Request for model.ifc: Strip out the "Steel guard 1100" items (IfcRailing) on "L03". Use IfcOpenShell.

First a look at what the model holds.

```python
import ifcopenshell
import ifcopenshell.util.element

model = ifcopenshell.open("model.ifc")
print(model.schema)
storey = next(s for s in model.by_type("IfcBuildingStorey") if s.Name == "L03")
railings = [e for e in ifcopenshell.util.element.get_decomposition(storey) if e.is_a("IfcRailing")]
seen = {}
for e in railings:
    element_type = ifcopenshell.util.element.get_type(e)
    name = element_type.Name if element_type not in (None, e) else None
    seen[name] = seen.get(name, 0) + 1
for name, count in sorted(seen.items(), key=str):
    print(count, "x", name)
```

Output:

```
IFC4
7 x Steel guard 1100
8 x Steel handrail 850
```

```python
import ifcopenshell
import ifcopenshell.api.root
import ifcopenshell.util.element

model = ifcopenshell.open("model.ifc")

storey = next(s for s in model.by_type("IfcBuildingStorey") if s.Name == "L03")
railings = [e for e in ifcopenshell.util.element.get_decomposition(storey) if e.is_a("IfcRailing")]
targets = [e for e in railings if (t := ifcopenshell.util.element.get_type(e)) not in (None, e) and t.Name == "Steel guard 1100"]

for e in targets:
    ifcopenshell.api.root.remove_product(model, product=e)
print(len(targets), "removed")

model.write("model_rev.ifc")
```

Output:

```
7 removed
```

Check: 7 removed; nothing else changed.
